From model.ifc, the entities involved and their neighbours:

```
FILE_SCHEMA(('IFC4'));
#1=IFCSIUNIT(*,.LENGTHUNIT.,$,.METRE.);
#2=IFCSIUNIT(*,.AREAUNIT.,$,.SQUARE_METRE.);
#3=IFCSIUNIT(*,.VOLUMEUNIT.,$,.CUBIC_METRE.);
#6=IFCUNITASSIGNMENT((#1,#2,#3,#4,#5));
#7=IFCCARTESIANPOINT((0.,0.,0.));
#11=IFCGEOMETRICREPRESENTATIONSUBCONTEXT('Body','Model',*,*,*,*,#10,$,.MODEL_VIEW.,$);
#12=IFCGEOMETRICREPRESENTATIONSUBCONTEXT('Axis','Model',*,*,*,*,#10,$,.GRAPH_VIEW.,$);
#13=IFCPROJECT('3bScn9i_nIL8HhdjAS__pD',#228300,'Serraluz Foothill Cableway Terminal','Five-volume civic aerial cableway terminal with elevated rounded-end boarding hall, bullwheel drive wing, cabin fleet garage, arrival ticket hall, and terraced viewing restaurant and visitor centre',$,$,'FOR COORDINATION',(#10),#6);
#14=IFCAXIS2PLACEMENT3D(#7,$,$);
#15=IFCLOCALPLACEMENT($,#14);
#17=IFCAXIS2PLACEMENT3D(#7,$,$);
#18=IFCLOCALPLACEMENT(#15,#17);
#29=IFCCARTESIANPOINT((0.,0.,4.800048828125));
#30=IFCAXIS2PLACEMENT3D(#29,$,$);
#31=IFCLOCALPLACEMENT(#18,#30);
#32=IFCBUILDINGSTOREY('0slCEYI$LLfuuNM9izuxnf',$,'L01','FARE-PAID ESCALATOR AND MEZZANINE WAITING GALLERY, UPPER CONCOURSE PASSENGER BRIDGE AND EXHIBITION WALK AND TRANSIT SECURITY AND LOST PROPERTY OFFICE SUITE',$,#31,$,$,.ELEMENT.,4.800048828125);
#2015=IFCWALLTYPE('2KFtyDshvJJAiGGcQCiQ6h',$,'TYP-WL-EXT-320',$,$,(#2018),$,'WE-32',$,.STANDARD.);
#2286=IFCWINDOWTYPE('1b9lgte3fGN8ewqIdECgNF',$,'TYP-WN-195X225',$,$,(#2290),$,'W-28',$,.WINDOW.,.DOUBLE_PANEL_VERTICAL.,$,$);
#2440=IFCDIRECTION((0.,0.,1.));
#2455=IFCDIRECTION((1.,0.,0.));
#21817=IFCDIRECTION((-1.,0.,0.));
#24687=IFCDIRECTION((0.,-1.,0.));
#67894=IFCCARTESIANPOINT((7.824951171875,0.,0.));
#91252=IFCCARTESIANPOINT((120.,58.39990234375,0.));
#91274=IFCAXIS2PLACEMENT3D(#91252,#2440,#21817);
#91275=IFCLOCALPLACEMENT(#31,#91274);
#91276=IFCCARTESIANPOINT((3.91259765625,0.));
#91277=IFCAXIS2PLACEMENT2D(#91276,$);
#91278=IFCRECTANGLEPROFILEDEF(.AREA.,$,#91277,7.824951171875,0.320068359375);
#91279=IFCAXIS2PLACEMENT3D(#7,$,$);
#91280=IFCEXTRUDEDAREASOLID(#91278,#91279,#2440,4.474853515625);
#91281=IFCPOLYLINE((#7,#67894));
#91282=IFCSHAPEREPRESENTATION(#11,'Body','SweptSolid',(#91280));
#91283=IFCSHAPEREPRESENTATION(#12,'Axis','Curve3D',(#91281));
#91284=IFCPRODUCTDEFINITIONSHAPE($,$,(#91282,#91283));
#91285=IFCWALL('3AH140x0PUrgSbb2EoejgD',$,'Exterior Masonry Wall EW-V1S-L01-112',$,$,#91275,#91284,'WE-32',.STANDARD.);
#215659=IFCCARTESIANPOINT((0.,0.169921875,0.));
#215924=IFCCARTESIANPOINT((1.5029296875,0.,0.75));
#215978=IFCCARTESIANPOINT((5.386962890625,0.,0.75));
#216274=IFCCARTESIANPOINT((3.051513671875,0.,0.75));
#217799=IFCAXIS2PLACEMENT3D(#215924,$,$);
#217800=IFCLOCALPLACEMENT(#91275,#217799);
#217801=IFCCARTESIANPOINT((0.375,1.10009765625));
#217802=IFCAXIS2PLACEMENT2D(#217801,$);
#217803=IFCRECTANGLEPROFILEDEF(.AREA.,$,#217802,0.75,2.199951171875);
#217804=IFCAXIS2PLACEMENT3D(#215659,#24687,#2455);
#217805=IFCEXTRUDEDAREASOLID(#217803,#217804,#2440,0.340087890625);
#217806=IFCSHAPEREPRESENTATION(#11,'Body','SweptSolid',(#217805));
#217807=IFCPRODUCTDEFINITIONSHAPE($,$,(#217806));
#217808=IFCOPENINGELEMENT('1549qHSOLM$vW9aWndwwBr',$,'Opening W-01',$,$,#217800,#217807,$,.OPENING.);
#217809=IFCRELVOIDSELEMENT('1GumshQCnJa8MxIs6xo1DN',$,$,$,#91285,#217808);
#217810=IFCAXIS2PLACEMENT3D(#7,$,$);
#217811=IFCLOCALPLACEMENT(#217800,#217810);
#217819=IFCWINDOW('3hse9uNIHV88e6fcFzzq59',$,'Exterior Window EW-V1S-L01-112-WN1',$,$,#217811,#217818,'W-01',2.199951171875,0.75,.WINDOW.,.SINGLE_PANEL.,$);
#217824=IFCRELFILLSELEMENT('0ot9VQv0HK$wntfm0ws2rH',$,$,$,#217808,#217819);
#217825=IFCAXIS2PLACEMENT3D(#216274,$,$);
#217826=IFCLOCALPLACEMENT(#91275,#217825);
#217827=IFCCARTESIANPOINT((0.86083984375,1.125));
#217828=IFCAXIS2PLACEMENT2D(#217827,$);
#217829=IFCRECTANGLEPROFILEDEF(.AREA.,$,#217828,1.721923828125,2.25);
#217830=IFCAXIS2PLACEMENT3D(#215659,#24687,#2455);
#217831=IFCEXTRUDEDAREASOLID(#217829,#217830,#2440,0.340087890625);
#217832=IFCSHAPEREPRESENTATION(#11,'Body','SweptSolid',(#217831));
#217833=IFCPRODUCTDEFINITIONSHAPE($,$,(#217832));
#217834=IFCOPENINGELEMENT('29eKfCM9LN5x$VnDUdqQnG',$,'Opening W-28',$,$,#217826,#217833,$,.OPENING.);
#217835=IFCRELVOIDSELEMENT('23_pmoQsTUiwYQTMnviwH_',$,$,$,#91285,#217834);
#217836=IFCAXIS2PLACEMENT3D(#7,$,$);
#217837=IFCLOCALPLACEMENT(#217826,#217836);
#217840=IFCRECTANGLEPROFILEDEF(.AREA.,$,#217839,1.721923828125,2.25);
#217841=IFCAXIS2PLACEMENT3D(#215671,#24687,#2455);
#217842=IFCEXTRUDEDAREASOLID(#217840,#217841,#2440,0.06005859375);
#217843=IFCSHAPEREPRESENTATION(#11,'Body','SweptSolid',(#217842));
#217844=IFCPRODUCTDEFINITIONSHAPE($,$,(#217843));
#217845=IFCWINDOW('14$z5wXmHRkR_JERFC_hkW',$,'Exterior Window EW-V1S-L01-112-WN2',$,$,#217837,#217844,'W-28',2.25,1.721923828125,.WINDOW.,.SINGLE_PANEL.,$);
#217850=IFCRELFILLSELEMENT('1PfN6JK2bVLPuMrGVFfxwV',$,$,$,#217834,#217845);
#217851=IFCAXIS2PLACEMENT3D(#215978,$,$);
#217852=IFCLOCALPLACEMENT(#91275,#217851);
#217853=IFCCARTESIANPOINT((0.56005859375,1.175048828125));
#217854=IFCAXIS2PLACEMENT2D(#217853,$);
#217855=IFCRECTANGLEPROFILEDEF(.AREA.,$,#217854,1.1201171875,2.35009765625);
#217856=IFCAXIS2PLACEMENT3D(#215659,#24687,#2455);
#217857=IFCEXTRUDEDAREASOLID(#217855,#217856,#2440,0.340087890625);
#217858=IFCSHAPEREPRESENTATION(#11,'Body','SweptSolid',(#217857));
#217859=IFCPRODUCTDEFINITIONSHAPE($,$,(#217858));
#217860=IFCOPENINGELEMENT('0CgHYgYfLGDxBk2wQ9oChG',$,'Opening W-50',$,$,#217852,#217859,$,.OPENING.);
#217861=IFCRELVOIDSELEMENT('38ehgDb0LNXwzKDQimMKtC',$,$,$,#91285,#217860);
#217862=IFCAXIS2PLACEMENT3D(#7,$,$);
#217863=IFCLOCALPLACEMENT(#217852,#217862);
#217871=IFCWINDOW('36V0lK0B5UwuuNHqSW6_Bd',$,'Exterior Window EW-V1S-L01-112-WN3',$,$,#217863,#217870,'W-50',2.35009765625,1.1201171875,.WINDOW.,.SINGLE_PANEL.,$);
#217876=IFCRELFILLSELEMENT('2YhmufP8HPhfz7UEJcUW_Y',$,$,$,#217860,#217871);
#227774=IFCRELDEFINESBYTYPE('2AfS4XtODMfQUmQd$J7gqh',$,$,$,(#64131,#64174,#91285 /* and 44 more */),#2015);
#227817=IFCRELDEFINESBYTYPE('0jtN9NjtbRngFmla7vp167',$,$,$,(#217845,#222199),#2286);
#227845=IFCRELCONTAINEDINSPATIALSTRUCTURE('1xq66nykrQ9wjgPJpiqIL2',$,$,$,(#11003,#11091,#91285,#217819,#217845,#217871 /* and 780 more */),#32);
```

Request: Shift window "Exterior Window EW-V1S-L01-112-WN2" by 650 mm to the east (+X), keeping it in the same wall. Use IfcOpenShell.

```python
import ifcopenshell
import ifcopenshell.api.geometry
import ifcopenshell.util.placement
import ifcopenshell.util.unit

model = ifcopenshell.open("model.ifc")
unit_scale = ifcopenshell.util.unit.calculate_unit_scale(model)

window = model.by_guid("14$z5wXmHRkR_JERFC_hkW")
opening = window.FillsVoids[0].RelatingOpeningElement
wall = opening.VoidsElements[0].RelatingBuildingElement

wall_matrix = ifcopenshell.util.placement.get_local_placement(wall.ObjectPlacement)
shift = wall_matrix[:3, 0] * -0.65 / unit_scale
before = ifcopenshell.util.placement.get_local_placement(window.ObjectPlacement)[:3, 3].copy()

# The window is placed relative to its opening, so it follows when the opening moves.
matrix = ifcopenshell.util.placement.get_local_placement(opening.ObjectPlacement)
matrix[:3, 3] += shift
ifcopenshell.api.geometry.edit_object_placement(
    model, product=opening, matrix=matrix, is_si=False, should_transform_children=True
)

after = ifcopenshell.util.placement.get_local_placement(window.ObjectPlacement)[:3, 3]
print("window moved by", (after - before).round(3) + 0.0)

model.write("model-out.ifc")
```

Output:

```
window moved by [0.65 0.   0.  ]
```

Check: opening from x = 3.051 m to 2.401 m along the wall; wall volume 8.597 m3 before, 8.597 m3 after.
